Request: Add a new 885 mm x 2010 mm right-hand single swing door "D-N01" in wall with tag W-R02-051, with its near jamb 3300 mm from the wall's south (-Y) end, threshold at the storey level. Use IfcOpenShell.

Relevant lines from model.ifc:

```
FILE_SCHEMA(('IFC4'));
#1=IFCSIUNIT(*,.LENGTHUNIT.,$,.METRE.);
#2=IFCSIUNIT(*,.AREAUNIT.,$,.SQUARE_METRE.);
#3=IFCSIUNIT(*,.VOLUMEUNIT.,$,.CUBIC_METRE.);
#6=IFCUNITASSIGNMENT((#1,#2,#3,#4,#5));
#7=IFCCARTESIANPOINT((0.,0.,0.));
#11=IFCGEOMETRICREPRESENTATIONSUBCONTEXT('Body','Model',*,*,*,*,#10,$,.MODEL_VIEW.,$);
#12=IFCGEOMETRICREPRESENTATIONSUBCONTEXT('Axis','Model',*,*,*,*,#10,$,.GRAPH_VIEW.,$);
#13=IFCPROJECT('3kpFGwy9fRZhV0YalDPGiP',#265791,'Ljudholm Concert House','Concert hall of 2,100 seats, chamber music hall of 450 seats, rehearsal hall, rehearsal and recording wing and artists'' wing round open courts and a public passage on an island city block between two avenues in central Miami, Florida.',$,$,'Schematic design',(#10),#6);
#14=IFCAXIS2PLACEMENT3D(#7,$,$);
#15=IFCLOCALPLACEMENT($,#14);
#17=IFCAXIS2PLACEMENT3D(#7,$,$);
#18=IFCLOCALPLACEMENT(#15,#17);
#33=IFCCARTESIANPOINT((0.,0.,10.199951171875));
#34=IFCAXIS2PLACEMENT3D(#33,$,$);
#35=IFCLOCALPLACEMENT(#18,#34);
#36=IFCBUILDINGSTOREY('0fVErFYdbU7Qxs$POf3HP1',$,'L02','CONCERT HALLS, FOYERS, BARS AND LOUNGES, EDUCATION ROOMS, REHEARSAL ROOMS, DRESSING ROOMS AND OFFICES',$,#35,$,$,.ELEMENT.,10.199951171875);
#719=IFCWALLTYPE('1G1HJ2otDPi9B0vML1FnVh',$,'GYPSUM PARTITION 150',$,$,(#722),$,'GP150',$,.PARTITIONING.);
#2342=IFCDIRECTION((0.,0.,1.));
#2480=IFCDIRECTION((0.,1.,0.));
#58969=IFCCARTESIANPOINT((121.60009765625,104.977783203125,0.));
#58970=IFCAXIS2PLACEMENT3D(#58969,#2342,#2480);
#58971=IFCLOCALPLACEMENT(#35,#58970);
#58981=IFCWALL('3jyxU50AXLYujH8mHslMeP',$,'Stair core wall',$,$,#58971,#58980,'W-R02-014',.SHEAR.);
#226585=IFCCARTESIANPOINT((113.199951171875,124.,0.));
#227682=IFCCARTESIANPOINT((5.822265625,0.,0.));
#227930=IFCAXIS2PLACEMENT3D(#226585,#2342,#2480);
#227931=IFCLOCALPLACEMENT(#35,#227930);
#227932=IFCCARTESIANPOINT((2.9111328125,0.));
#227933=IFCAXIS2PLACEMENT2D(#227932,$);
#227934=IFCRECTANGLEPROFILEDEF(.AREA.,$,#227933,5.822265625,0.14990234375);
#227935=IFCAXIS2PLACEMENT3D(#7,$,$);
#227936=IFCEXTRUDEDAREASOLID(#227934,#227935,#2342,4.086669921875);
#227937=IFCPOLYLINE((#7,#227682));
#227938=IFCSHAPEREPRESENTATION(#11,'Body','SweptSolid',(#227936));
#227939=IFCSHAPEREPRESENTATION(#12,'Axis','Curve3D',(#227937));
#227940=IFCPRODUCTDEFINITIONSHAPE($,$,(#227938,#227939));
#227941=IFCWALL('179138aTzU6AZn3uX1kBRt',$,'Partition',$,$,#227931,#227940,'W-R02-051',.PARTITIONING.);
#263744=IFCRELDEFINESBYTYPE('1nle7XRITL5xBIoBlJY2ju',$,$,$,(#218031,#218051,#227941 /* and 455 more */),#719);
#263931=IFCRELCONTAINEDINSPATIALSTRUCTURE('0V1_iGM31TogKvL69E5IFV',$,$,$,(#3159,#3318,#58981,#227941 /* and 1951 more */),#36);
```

```python
import numpy as np
import ifcopenshell
import ifcopenshell.api.feature
import ifcopenshell.api.geometry
import ifcopenshell.api.root
import ifcopenshell.api.spatial
import ifcopenshell.geom
import ifcopenshell.util.element
import ifcopenshell.util.placement
import ifcopenshell.util.representation
import ifcopenshell.util.shape
import ifcopenshell.util.unit

model = ifcopenshell.open("model.ifc")
unit_scale = ifcopenshell.util.unit.calculate_unit_scale(model)
settings = ifcopenshell.geom.settings()


def volume(element):
    """Net volume in cubic metres, openings subtracted."""
    shape = ifcopenshell.geom.create_shape(settings, element)
    return ifcopenshell.util.shape.get_volume(shape.geometry)


wall = model.by_id(227941)
storey = ifcopenshell.util.element.get_container(wall, ifc_class="IfcBuildingStorey")
context = ifcopenshell.util.representation.get_context(model, "Model", "Body", "MODEL_VIEW")
before = volume(wall)

width, height, from_end, sill = 0.885, 2.01, 3.3, 0.0  # metres

# The wall runs along its own X axis, and the end named is its -X end.
wall_shape = ifcopenshell.geom.create_shape(settings, wall)
x, y, z = ifcopenshell.util.shape.get_vertices(wall_shape.geometry).T
start = x.min() + from_end
face, thickness = float(y.min()), float(y.max() - y.min())
wall_matrix = ifcopenshell.util.placement.get_local_placement(wall.ObjectPlacement)
level = ifcopenshell.util.placement.get_local_placement(storey.ObjectPlacement)[2, 3]


def in_wall(x, y):
    """Placement at x, y metres in the wall's axes, at sill height."""
    matrix = wall_matrix.copy()
    matrix[:, 3] = wall_matrix @ np.array([x / unit_scale, y / unit_scale, 0.0, 1.0])
    matrix[2, 3] = level + sill / unit_scale
    return matrix


# Opening: a box that overshoots both wall faces by 50 mm.
opening = ifcopenshell.api.root.create_entity(model, ifc_class="IfcOpeningElement", predefined_type="OPENING")
box = ifcopenshell.api.geometry.add_wall_representation(
    model, context=context, length=width, height=height, thickness=thickness + 0.1
)
ifcopenshell.api.geometry.assign_representation(model, product=opening, representation=box)
ifcopenshell.api.geometry.edit_object_placement(model, product=opening, matrix=in_wall(start, face - 0.05), is_si=False)
ifcopenshell.api.feature.add_feature(model, feature=opening, element=wall)

door = ifcopenshell.api.root.create_entity(model, ifc_class="IfcDoor", name="D-N01", predefined_type="DOOR")
door.OverallWidth, door.OverallHeight = width / unit_scale, height / unit_scale
door.OperationType = "SINGLE_SWING_RIGHT"
body = ifcopenshell.api.geometry.add_door_representation(
    model,
    context=context,
    overall_width=door.OverallWidth,
    overall_height=door.OverallHeight,
    operation_type="SINGLE_SWING_RIGHT",
    lining_properties={"LiningDepth": thickness / unit_scale, "ThresholdDepth": thickness / unit_scale},
)
ifcopenshell.api.geometry.assign_representation(model, product=door, representation=body)
ifcopenshell.api.spatial.assign_container(model, products=[door], relating_structure=storey)
ifcopenshell.api.feature.add_filling(model, opening=opening, element=door)

# The lining spans the wall, so the door starts at the wall face.
ifcopenshell.api.geometry.edit_object_placement(model, product=door, matrix=in_wall(start, face), is_si=False)

after = volume(wall)

print(f"wall volume {before:.3f} -> {after:.3f} m3")

model.write("model_v2.ifc")
```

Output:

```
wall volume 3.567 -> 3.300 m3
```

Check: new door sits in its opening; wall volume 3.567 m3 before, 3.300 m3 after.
